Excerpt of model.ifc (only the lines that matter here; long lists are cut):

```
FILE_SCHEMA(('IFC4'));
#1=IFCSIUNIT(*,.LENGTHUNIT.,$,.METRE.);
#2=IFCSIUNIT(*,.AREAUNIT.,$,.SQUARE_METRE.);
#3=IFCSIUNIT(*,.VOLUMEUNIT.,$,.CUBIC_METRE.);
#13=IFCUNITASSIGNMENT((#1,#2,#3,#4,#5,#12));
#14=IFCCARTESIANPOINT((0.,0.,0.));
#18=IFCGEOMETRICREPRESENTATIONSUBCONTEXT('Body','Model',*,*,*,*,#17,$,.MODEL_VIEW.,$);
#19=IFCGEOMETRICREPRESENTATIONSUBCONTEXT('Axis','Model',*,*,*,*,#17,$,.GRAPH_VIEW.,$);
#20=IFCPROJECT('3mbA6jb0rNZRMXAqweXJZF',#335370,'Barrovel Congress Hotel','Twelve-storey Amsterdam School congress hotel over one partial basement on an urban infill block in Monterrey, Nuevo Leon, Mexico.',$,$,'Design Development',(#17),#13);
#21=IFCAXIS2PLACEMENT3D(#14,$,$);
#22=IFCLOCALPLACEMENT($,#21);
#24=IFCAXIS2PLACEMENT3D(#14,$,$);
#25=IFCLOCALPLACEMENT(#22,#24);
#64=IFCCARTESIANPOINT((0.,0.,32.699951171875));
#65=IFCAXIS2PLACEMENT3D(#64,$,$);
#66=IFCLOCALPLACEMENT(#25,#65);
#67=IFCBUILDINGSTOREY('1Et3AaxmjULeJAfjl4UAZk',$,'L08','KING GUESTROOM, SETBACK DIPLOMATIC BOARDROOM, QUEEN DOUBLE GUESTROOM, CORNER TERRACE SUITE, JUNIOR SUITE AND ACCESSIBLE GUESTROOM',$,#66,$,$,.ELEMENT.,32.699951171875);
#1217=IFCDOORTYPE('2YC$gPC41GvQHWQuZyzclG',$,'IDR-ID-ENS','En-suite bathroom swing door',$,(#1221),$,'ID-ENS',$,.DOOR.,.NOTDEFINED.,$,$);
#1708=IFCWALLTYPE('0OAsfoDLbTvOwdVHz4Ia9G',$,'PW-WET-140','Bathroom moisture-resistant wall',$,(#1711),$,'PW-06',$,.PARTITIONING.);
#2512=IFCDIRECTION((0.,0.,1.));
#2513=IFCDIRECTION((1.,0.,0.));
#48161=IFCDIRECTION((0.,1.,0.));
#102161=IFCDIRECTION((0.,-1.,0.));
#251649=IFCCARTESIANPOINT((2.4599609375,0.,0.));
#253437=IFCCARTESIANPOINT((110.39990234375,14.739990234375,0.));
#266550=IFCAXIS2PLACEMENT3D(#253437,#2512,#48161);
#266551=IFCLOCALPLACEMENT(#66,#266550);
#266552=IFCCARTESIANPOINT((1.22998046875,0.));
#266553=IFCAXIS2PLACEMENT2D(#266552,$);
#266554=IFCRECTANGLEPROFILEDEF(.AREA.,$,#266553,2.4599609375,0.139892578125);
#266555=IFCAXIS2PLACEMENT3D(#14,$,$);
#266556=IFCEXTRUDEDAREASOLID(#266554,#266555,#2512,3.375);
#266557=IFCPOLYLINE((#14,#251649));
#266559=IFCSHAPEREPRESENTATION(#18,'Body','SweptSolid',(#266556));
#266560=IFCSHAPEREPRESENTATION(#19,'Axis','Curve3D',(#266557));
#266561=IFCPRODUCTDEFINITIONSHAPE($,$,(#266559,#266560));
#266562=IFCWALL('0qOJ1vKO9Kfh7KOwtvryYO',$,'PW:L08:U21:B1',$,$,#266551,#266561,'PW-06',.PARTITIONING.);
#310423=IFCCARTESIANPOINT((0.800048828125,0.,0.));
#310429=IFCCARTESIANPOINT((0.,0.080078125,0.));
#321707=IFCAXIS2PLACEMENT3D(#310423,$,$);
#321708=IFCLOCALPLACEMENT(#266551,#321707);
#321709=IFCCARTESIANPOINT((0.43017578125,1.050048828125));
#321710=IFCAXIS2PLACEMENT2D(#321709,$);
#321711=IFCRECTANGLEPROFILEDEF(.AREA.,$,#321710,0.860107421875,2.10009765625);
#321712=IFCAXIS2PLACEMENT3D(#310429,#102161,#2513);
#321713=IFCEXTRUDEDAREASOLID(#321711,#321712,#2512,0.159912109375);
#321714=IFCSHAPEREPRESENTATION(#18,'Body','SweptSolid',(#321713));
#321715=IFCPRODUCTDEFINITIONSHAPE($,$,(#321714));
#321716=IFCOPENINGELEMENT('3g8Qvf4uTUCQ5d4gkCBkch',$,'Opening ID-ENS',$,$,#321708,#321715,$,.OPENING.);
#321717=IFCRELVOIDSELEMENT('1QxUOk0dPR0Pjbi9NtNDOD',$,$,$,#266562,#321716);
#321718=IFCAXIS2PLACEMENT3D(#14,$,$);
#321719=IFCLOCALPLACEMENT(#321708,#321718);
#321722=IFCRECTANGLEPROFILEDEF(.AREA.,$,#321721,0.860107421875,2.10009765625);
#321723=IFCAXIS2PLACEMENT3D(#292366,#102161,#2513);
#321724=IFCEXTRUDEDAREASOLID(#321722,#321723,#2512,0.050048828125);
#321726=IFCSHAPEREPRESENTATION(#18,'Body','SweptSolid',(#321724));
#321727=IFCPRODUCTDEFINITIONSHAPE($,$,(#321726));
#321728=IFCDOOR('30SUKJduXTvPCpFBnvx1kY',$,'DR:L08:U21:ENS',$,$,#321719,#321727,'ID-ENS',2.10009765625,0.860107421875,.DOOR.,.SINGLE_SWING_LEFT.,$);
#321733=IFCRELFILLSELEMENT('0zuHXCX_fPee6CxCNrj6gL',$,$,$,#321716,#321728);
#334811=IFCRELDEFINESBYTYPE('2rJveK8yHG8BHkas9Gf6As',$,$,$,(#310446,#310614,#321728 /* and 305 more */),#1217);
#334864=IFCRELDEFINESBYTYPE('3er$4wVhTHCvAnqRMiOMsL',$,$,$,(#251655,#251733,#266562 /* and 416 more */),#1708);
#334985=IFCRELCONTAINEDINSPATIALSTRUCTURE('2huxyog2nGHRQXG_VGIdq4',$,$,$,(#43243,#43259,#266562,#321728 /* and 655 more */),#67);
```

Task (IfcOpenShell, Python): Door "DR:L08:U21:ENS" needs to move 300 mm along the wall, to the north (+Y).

```python
import ifcopenshell
import ifcopenshell.api.geometry
import ifcopenshell.util.placement
import ifcopenshell.util.unit

model = ifcopenshell.open("model.ifc")
unit_scale = ifcopenshell.util.unit.calculate_unit_scale(model)

door = model.by_guid("30SUKJduXTvPCpFBnvx1kY")
opening = door.FillsVoids[0].RelatingOpeningElement
wall = opening.VoidsElements[0].RelatingBuildingElement

wall_matrix = ifcopenshell.util.placement.get_local_placement(wall.ObjectPlacement)
shift = wall_matrix[:3, 0] * 0.3 / unit_scale
before = ifcopenshell.util.placement.get_local_placement(door.ObjectPlacement)[:3, 3].copy()

# The door is placed relative to its opening, so it follows when the opening moves.
matrix = ifcopenshell.util.placement.get_local_placement(opening.ObjectPlacement)
matrix[:3, 3] += shift
ifcopenshell.api.geometry.edit_object_placement(
    model, product=opening, matrix=matrix, is_si=False, should_transform_children=True
)

after = ifcopenshell.util.placement.get_local_placement(door.ObjectPlacement)[:3, 3]
print("door moved by", (after - before).round(3) + 0.0)

model.write("model-out.ifc")
```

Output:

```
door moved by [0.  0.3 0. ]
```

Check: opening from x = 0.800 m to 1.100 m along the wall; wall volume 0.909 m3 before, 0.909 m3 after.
